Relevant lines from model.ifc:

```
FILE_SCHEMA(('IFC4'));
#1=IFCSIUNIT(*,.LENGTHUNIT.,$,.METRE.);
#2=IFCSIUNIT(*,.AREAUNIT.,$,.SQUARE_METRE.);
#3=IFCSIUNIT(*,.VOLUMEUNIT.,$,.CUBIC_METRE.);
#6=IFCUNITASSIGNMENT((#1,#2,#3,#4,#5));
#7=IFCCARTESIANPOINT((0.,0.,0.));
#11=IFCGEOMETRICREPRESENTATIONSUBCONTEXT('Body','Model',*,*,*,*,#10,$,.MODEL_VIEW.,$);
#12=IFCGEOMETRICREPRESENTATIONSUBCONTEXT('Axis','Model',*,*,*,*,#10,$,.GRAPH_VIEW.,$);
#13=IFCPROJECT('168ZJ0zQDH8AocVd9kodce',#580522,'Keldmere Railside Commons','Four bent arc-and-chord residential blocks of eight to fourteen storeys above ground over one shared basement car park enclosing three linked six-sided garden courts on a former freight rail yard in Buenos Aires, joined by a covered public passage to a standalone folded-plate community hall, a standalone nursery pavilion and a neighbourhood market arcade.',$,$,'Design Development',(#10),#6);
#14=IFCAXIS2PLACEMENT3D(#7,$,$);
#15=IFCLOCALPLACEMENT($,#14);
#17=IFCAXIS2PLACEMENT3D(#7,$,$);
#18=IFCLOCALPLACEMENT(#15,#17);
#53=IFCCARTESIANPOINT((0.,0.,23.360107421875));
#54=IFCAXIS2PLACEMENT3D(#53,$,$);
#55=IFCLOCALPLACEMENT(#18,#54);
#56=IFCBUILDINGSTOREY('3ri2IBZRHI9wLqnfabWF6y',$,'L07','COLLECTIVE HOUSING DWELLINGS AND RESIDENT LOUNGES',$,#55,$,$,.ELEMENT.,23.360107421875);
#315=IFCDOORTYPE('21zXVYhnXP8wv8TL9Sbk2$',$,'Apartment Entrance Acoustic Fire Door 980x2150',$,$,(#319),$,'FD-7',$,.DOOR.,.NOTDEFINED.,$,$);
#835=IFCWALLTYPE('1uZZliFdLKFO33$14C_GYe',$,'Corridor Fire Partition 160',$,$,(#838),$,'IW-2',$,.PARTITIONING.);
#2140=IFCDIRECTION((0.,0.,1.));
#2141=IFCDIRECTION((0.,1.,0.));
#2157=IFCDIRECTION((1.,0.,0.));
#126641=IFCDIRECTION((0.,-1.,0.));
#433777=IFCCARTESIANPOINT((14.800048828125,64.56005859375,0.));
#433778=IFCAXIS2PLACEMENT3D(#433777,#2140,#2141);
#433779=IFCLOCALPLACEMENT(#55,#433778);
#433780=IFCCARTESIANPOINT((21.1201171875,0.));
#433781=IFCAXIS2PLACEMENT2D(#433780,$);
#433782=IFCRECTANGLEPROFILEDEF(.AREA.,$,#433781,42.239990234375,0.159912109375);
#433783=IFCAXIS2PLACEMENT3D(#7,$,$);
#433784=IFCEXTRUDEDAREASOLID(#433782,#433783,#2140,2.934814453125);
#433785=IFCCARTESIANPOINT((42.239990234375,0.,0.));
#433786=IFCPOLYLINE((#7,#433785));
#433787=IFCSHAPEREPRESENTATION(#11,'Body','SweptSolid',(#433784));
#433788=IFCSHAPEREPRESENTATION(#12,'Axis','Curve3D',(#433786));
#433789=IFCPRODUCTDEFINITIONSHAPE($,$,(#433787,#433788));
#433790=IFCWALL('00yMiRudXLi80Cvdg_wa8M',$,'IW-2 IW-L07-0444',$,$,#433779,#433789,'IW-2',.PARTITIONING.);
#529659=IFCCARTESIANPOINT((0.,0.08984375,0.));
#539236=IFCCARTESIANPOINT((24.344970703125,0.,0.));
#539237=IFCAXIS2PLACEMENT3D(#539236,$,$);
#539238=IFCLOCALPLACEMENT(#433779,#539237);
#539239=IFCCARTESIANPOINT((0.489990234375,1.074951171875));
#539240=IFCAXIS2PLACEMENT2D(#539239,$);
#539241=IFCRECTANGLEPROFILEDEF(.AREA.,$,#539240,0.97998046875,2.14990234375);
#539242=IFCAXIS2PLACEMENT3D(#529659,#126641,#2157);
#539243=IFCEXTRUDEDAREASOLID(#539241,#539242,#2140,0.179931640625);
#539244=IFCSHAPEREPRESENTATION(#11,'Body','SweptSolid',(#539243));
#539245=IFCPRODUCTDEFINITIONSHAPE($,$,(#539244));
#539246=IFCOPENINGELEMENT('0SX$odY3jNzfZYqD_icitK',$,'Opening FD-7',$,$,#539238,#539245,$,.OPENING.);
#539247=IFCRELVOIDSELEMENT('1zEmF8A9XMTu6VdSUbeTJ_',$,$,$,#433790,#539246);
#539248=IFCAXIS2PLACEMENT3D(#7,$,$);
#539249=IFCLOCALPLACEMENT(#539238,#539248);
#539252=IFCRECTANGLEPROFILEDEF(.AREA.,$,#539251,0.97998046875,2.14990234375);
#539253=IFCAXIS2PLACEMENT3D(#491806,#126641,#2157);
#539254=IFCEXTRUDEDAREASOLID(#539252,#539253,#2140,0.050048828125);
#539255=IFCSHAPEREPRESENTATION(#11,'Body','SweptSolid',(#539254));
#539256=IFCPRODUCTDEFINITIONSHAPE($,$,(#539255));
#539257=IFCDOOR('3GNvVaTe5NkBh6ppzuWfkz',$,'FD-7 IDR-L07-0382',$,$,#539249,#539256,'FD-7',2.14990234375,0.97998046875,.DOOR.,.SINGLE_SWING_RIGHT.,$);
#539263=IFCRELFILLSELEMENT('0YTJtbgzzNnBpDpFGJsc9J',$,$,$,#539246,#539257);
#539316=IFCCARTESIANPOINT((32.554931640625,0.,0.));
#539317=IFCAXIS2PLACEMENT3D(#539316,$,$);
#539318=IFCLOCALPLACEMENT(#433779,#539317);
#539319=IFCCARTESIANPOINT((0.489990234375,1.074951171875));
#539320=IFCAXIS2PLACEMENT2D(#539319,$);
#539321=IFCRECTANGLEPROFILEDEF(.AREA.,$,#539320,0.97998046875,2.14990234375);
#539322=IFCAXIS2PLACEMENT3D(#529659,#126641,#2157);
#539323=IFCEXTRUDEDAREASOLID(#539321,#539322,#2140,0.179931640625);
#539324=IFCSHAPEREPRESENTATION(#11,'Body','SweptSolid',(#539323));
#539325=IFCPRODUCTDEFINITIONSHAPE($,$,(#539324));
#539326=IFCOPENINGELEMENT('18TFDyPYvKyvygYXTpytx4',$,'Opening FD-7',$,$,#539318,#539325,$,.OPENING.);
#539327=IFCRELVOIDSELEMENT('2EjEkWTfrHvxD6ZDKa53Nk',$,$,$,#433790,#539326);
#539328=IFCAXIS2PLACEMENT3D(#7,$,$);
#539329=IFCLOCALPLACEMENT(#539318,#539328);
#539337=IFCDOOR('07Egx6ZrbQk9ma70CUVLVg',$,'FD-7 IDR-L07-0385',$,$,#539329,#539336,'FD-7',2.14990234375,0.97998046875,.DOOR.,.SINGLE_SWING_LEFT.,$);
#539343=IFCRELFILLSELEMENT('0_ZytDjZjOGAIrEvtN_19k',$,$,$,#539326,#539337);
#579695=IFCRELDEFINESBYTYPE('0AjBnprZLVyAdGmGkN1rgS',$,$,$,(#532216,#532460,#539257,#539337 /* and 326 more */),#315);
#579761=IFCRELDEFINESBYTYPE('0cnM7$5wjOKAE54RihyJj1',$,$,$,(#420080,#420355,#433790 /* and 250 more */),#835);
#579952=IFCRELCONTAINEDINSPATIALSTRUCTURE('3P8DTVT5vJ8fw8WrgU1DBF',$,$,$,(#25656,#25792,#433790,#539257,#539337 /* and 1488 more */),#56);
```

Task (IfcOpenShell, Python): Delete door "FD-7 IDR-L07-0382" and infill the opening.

```python
import ifcopenshell
import ifcopenshell.api.feature
import ifcopenshell.api.root
import ifcopenshell.geom
import ifcopenshell.util.shape

model = ifcopenshell.open("model.ifc")
settings = ifcopenshell.geom.settings()


def volume(element):
    """Net volume in cubic metres, openings subtracted."""
    shape = ifcopenshell.geom.create_shape(settings, element)
    return ifcopenshell.util.shape.get_volume(shape.geometry)


door = model.by_guid("3GNvVaTe5NkBh6ppzuWfkz")
opening = door.FillsVoids[0].RelatingOpeningElement
wall = opening.VoidsElements[0].RelatingBuildingElement
before = volume(wall)

ifcopenshell.api.root.remove_product(model, product=door)
ifcopenshell.api.feature.remove_feature(model, feature=opening)

after = volume(wall)

print(f"wall volume {before:.3f} -> {after:.3f} m3")

model.write("model_edited.ifc")
```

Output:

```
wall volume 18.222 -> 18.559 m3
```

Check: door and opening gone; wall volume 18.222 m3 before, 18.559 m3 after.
